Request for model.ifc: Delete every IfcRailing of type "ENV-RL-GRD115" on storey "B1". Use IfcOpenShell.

First a look at what the model holds.

```python
import ifcopenshell
import ifcopenshell.util.element

model = ifcopenshell.open("model.ifc")
print(model.schema)
storey = next(s for s in model.by_type("IfcBuildingStorey") if s.Name == "B1")
railings = [e for e in ifcopenshell.util.element.get_decomposition(storey) if e.is_a("IfcRailing")]
seen = {}
for e in railings:
    element_type = ifcopenshell.util.element.get_type(e)
    name = element_type.Name if element_type not in (None, e) else None
    seen[name] = seen.get(name, 0) + 1
for name, count in sorted(seen.items(), key=str):
    print(count, "x", name)
```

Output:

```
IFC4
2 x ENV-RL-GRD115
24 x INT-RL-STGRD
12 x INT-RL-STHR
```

```python
import ifcopenshell
import ifcopenshell.api.root
import ifcopenshell.util.element

model = ifcopenshell.open("model.ifc")

storey = next(s for s in model.by_type("IfcBuildingStorey") if s.Name == "B1")
railings = [e for e in ifcopenshell.util.element.get_decomposition(storey) if e.is_a("IfcRailing")]
targets = [e for e in railings if (t := ifcopenshell.util.element.get_type(e)) not in (None, e) and t.Name == "ENV-RL-GRD115"]

for e in targets:
    ifcopenshell.api.root.remove_product(model, product=e)
print(len(targets), "removed")

model.write("model_v2.ifc")
```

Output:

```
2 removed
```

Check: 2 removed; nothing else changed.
